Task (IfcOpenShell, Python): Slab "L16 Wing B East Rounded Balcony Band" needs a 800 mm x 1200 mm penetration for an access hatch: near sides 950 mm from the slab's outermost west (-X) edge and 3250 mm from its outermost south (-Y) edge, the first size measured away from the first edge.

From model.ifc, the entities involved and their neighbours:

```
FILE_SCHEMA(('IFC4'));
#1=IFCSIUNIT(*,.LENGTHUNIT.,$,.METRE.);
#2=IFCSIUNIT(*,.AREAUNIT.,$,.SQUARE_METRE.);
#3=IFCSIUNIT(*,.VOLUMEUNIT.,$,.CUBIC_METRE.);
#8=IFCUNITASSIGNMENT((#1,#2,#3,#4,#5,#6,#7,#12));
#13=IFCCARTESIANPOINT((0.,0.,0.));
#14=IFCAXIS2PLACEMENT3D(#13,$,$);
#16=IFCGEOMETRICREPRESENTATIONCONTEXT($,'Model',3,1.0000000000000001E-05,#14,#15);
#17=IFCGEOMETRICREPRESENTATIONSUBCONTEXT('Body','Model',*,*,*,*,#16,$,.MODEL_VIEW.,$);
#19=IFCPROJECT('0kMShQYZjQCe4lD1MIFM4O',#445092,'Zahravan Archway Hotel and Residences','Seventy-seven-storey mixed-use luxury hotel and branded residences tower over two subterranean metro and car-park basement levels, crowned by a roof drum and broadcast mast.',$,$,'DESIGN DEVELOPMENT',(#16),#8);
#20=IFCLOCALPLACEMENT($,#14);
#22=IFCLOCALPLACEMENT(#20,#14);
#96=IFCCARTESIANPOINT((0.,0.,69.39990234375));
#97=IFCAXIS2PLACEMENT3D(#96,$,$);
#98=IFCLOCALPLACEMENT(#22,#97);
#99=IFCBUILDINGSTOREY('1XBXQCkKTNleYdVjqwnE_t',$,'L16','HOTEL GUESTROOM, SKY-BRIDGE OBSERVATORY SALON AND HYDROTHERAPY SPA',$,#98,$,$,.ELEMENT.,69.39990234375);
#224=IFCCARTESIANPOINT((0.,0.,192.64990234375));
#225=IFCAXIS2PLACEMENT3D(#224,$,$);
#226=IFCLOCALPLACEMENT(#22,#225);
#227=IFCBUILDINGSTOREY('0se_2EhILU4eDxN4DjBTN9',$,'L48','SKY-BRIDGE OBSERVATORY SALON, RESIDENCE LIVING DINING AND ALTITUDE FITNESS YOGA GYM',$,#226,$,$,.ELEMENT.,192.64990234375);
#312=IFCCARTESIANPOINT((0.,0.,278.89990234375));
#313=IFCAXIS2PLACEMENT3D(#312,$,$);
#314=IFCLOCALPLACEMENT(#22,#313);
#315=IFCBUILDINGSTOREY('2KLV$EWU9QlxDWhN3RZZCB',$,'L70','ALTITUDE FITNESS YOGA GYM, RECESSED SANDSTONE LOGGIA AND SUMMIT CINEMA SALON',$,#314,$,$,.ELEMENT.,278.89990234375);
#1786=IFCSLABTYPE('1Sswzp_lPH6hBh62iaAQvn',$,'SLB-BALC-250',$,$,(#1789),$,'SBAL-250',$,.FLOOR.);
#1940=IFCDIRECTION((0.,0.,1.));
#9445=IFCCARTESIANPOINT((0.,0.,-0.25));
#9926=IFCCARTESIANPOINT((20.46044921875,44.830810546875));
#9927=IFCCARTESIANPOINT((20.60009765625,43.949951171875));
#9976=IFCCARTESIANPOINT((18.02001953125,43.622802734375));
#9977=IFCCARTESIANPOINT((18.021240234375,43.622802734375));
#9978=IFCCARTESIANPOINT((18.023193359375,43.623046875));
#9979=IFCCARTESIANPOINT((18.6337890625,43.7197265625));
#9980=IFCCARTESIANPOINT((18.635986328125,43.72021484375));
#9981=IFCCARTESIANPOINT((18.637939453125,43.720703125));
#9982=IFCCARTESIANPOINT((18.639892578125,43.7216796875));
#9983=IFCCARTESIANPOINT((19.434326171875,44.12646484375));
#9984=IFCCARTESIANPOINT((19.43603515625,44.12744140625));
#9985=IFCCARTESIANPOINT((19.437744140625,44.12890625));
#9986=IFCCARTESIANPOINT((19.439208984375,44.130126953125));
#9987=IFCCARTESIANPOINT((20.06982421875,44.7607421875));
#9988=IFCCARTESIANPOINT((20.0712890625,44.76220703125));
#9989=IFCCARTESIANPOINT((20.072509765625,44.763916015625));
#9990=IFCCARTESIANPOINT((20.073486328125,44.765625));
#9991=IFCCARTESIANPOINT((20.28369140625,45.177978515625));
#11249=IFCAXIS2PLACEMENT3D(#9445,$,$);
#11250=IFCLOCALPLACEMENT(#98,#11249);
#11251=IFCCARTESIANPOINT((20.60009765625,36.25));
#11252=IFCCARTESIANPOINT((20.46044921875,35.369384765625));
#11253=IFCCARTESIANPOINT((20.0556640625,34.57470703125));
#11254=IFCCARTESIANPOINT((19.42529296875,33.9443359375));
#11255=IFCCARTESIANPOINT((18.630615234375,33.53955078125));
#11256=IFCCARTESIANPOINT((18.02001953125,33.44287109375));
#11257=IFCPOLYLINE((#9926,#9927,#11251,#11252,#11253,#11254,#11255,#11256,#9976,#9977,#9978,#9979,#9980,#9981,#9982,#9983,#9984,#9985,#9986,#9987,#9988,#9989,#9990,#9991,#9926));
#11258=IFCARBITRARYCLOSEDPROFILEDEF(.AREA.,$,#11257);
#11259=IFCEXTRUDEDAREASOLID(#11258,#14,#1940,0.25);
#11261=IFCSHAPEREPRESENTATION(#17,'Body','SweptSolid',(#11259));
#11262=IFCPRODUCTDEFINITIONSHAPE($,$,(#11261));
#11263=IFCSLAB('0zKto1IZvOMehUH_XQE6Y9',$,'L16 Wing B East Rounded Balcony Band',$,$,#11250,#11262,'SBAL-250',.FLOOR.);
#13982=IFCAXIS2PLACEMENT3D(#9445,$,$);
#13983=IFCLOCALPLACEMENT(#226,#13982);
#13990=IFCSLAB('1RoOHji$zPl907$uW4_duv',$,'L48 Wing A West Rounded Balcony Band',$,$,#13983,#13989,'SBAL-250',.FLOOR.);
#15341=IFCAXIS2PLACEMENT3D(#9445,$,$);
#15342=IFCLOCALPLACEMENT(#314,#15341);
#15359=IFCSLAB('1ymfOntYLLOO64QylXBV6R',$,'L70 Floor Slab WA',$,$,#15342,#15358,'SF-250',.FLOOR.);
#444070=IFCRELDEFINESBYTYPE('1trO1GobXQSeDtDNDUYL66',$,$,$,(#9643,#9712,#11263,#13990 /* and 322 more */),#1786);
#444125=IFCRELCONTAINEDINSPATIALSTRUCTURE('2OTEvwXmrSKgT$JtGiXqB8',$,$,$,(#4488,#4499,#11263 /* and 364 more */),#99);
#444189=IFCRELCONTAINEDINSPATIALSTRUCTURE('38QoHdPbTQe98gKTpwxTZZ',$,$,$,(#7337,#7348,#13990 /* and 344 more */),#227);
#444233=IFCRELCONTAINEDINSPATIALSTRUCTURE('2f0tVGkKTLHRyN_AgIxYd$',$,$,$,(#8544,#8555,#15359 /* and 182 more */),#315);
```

```python
import numpy as np
import ifcopenshell
import ifcopenshell.api.feature
import ifcopenshell.api.geometry
import ifcopenshell.api.root
import ifcopenshell.geom
import ifcopenshell.util.placement
import ifcopenshell.util.representation
import ifcopenshell.util.shape
import ifcopenshell.util.unit

model = ifcopenshell.open("model.ifc")
unit_scale = ifcopenshell.util.unit.calculate_unit_scale(model)
settings = ifcopenshell.geom.settings()


def volume(element):
    """Net volume in cubic metres, openings subtracted."""
    shape = ifcopenshell.geom.create_shape(settings, element)
    return ifcopenshell.util.shape.get_volume(shape.geometry)


slab = model.by_guid("0zKto1IZvOMehUH_XQE6Y9")
before = volume(slab)

# Extent in the slab's own axes, in metres. The edges named are its -X and -Y sides.
slab_shape = ifcopenshell.geom.create_shape(settings, slab)
vertices = ifcopenshell.util.shape.get_vertices(slab_shape.geometry)
x_min, y_min, bottom = vertices.min(axis=0)
top = vertices[:, 2].max()

opening = ifcopenshell.api.root.create_entity(model, ifc_class="IfcOpeningElement", name="Access hatch opening", predefined_type="OPENING")
context = ifcopenshell.util.representation.get_context(model, "Model", "Body", "MODEL_VIEW")
width, depth = 0.8, 1.2
outline = [(0.0, 0.0), (width, 0.0), (width, depth), (0.0, depth), (0.0, 0.0)]
# Overshoot both faces by 50 mm so the cut is clean.
shape = ifcopenshell.api.geometry.add_slab_representation(
    model, context=context, depth=top - bottom + 0.1, polyline=outline
)
ifcopenshell.api.geometry.assign_representation(model, product=opening, representation=shape)

matrix = ifcopenshell.util.placement.get_local_placement(slab.ObjectPlacement)
matrix[:, 3] = matrix @ np.append(np.array([x_min + 0.95, y_min + 3.25, bottom - 0.05]) / unit_scale, 1.0)
ifcopenshell.api.geometry.edit_object_placement(model, product=opening, matrix=matrix, is_si=False)
ifcopenshell.api.feature.add_feature(model, feature=opening, element=slab)

after = volume(slab)

print(f"slab volume {before:.3f} -> {after:.3f} m3")

model.write("model_v2.ifc")
```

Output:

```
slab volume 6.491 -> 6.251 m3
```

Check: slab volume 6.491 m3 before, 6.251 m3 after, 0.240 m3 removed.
